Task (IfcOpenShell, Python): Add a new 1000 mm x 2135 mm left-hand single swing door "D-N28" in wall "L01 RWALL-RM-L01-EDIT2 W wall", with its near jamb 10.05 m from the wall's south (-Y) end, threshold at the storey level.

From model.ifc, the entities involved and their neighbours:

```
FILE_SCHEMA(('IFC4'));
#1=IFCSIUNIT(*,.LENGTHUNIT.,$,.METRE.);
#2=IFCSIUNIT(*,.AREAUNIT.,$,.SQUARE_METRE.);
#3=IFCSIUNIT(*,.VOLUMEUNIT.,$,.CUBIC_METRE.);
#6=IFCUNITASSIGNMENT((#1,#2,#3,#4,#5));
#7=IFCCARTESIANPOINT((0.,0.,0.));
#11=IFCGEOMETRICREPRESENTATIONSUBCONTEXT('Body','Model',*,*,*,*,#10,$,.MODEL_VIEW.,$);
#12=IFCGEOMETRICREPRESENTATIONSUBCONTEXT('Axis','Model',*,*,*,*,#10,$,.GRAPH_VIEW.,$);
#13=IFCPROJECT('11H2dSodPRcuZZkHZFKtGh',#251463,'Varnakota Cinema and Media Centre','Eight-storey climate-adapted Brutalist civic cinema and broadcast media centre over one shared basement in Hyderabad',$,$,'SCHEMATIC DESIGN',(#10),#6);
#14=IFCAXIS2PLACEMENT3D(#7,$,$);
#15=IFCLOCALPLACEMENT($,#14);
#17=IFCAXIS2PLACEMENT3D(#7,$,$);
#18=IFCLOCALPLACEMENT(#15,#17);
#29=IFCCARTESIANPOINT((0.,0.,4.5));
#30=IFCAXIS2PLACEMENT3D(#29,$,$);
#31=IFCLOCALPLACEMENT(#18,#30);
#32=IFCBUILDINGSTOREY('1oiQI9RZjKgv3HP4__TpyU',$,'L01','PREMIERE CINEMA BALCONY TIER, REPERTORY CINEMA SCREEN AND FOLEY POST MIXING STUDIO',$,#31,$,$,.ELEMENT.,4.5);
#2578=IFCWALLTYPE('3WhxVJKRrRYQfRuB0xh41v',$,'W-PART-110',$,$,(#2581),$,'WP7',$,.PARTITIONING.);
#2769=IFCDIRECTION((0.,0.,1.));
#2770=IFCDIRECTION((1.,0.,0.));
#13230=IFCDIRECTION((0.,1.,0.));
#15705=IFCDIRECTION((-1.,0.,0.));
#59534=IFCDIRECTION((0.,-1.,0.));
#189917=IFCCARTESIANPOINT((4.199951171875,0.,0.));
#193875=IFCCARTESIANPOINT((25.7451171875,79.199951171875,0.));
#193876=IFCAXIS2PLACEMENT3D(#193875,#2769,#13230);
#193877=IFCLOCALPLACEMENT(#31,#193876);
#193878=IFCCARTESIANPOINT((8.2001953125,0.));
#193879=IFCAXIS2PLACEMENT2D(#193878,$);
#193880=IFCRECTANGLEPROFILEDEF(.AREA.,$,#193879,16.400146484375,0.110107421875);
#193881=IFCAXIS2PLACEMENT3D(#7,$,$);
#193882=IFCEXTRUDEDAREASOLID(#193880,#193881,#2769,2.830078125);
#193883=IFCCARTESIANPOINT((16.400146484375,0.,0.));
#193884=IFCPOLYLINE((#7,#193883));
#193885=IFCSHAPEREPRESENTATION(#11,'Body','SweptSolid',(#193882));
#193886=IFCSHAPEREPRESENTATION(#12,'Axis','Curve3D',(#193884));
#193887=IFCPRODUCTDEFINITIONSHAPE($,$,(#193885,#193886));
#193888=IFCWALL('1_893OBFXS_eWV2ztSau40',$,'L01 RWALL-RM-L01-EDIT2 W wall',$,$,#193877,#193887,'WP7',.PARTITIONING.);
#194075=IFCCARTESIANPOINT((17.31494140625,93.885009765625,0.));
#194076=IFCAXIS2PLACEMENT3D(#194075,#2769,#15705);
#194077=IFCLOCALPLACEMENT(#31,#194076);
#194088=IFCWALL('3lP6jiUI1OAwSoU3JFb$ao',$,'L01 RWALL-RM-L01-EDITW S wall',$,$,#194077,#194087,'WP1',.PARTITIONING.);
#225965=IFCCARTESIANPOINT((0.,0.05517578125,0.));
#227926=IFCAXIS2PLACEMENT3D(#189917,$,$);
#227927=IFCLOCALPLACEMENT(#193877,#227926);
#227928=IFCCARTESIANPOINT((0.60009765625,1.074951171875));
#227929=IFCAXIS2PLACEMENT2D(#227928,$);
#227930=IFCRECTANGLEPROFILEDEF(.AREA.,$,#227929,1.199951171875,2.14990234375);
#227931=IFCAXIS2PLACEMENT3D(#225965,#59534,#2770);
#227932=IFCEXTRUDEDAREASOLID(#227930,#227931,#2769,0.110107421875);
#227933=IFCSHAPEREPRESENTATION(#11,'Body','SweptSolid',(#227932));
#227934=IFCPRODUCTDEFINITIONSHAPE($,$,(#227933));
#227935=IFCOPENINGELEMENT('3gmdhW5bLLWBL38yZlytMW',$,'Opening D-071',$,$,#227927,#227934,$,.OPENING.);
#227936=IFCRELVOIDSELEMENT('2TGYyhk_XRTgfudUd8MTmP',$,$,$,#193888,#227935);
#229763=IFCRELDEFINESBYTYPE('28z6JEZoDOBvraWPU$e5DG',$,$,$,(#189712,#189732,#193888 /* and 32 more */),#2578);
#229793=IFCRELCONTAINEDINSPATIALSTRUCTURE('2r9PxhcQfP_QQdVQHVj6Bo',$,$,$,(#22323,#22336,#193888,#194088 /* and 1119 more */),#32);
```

```python
import numpy as np
import ifcopenshell
import ifcopenshell.api.feature
import ifcopenshell.api.geometry
import ifcopenshell.api.root
import ifcopenshell.api.spatial
import ifcopenshell.geom
import ifcopenshell.util.element
import ifcopenshell.util.placement
import ifcopenshell.util.representation
import ifcopenshell.util.shape
import ifcopenshell.util.unit

model = ifcopenshell.open("model.ifc")
unit_scale = ifcopenshell.util.unit.calculate_unit_scale(model)
settings = ifcopenshell.geom.settings()


def volume(element):
    """Net volume in cubic metres, openings subtracted."""
    shape = ifcopenshell.geom.create_shape(settings, element)
    return ifcopenshell.util.shape.get_volume(shape.geometry)


wall = model.by_id(193888)
storey = ifcopenshell.util.element.get_container(wall, ifc_class="IfcBuildingStorey")
context = ifcopenshell.util.representation.get_context(model, "Model", "Body", "MODEL_VIEW")
before = volume(wall)

width, height, from_end, sill = 1, 2.135, 10.05, 0.0  # metres

# The wall runs along its own X axis, and the end named is its -X end.
wall_shape = ifcopenshell.geom.create_shape(settings, wall)
x, y, z = ifcopenshell.util.shape.get_vertices(wall_shape.geometry).T
start = x.min() + from_end
face, thickness = float(y.min()), float(y.max() - y.min())
wall_matrix = ifcopenshell.util.placement.get_local_placement(wall.ObjectPlacement)
level = ifcopenshell.util.placement.get_local_placement(storey.ObjectPlacement)[2, 3]


def in_wall(x, y):
    """Placement at x, y metres in the wall's axes, at sill height."""
    matrix = wall_matrix.copy()
    matrix[:, 3] = wall_matrix @ np.array([x / unit_scale, y / unit_scale, 0.0, 1.0])
    matrix[2, 3] = level + sill / unit_scale
    return matrix


# Opening: a box that overshoots both wall faces by 50 mm.
opening = ifcopenshell.api.root.create_entity(model, ifc_class="IfcOpeningElement", predefined_type="OPENING")
box = ifcopenshell.api.geometry.add_wall_representation(
    model, context=context, length=width, height=height, thickness=thickness + 0.1
)
ifcopenshell.api.geometry.assign_representation(model, product=opening, representation=box)
ifcopenshell.api.geometry.edit_object_placement(model, product=opening, matrix=in_wall(start, face - 0.05), is_si=False)
ifcopenshell.api.feature.add_feature(model, feature=opening, element=wall)

door = ifcopenshell.api.root.create_entity(model, ifc_class="IfcDoor", name="D-N28", predefined_type="DOOR")
door.OverallWidth, door.OverallHeight = width / unit_scale, height / unit_scale
door.OperationType = "SINGLE_SWING_LEFT"
body = ifcopenshell.api.geometry.add_door_representation(
    model,
    context=context,
    overall_width=door.OverallWidth,
    overall_height=door.OverallHeight,
    operation_type="SINGLE_SWING_LEFT",
    lining_properties={"LiningDepth": thickness / unit_scale, "ThresholdDepth": thickness / unit_scale},
)
ifcopenshell.api.geometry.assign_representation(model, product=door, representation=body)
ifcopenshell.api.spatial.assign_container(model, products=[door], relating_structure=storey)
ifcopenshell.api.feature.add_filling(model, opening=opening, element=door)

# The lining spans the wall, so the door starts at the wall face.
ifcopenshell.api.geometry.edit_object_placement(model, product=door, matrix=in_wall(start, face), is_si=False)

after = volume(wall)

print(f"wall volume {before:.3f} -> {after:.3f} m3")

model.write("model_v2.ifc")
```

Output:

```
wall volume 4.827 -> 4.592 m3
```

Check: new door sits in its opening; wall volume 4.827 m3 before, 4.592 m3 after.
